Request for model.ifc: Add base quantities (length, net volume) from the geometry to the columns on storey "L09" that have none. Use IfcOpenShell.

First a look at what the model holds.

```python
import ifcopenshell
import ifcopenshell.util.element
import ifcopenshell.util.unit

model = ifcopenshell.open("model.ifc")
print(model.schema)
for unit_type in ("LENGTHUNIT", "AREAUNIT", "VOLUMEUNIT"):
    print(unit_type, ifcopenshell.util.unit.calculate_unit_scale(model, unit_type))
storey = next(s for s in model.by_type("IfcBuildingStorey") if s.Name == "L09")
columns = [e for e in ifcopenshell.util.element.get_decomposition(storey) if e.is_a("IfcColumn")]
for e in sorted(columns, key=lambda e: e.id()):
    print(e.id(), e.is_a(), e.Name, list(ifcopenshell.util.element.get_psets(e, qtos_only=True)), sep=" | ")
```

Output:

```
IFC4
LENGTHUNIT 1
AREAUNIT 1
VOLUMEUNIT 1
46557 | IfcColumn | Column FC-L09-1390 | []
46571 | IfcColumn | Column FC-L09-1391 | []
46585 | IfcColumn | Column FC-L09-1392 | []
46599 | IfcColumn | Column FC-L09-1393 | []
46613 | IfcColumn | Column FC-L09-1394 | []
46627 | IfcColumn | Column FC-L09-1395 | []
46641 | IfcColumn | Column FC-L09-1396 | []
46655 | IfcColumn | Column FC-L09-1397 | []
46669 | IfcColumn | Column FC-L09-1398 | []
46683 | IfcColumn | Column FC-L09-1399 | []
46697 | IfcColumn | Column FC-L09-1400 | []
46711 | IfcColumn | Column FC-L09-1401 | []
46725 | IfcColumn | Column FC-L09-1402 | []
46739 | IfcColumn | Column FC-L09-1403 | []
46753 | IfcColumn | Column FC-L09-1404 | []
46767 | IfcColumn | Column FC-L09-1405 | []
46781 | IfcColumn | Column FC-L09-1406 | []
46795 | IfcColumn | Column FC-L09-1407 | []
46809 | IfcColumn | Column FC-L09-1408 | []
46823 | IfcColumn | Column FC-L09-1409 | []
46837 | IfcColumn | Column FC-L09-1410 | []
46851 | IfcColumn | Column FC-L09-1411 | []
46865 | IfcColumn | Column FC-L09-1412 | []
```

```python
import ifcopenshell
import ifcopenshell.api.pset
import ifcopenshell.geom
import ifcopenshell.util.element
import ifcopenshell.util.shape
import ifcopenshell.util.unit

model = ifcopenshell.open("model.ifc")
unit_scale = ifcopenshell.util.unit.calculate_unit_scale(model)
volume_scale = ifcopenshell.util.unit.calculate_unit_scale(model, "VOLUMEUNIT")
settings = ifcopenshell.geom.settings()

storey = next(s for s in model.by_type("IfcBuildingStorey") if s.Name == "L09")
columns = [e for e in ifcopenshell.util.element.get_decomposition(storey) if e.is_a("IfcColumn")]

for e in sorted(columns, key=lambda e: e.id()):
    if ifcopenshell.util.element.get_psets(e, qtos_only=True, should_inherit=False):
        continue
    # Geometry comes back in metres, in the element's own axes.
    shape = ifcopenshell.geom.create_shape(settings, e)
    values = {
        "Length": ifcopenshell.util.shape.get_z(shape.geometry) / unit_scale,
        "NetVolume": ifcopenshell.util.shape.get_volume(shape.geometry) / volume_scale,
    }
    qto = ifcopenshell.api.pset.add_qto(model, product=e, name="Qto_ColumnBaseQuantities")
    ifcopenshell.api.pset.edit_qto(model, qto=qto, properties=values)
    print(e.id(), {k: round(v, 3) for k, v in values.items()})

model.write("model_updated.ifc")
```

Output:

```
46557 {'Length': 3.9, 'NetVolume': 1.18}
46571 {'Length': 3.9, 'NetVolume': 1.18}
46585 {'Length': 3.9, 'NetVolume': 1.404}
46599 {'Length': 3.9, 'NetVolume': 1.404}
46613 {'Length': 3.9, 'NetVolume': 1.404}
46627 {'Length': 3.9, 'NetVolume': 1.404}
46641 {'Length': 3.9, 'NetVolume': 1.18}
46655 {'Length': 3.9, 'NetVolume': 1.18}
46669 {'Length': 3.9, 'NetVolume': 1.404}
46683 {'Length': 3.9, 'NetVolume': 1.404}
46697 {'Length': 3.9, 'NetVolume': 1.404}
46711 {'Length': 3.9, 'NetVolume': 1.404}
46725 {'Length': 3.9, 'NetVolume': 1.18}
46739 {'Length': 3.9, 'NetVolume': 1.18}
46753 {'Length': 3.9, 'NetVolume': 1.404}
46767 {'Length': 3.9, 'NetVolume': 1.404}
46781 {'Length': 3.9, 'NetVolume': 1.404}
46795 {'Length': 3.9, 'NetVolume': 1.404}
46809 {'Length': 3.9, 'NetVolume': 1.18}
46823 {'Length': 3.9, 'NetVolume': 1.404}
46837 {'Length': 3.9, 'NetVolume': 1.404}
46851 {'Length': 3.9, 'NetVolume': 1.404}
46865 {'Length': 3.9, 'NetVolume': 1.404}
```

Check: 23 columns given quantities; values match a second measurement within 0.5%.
